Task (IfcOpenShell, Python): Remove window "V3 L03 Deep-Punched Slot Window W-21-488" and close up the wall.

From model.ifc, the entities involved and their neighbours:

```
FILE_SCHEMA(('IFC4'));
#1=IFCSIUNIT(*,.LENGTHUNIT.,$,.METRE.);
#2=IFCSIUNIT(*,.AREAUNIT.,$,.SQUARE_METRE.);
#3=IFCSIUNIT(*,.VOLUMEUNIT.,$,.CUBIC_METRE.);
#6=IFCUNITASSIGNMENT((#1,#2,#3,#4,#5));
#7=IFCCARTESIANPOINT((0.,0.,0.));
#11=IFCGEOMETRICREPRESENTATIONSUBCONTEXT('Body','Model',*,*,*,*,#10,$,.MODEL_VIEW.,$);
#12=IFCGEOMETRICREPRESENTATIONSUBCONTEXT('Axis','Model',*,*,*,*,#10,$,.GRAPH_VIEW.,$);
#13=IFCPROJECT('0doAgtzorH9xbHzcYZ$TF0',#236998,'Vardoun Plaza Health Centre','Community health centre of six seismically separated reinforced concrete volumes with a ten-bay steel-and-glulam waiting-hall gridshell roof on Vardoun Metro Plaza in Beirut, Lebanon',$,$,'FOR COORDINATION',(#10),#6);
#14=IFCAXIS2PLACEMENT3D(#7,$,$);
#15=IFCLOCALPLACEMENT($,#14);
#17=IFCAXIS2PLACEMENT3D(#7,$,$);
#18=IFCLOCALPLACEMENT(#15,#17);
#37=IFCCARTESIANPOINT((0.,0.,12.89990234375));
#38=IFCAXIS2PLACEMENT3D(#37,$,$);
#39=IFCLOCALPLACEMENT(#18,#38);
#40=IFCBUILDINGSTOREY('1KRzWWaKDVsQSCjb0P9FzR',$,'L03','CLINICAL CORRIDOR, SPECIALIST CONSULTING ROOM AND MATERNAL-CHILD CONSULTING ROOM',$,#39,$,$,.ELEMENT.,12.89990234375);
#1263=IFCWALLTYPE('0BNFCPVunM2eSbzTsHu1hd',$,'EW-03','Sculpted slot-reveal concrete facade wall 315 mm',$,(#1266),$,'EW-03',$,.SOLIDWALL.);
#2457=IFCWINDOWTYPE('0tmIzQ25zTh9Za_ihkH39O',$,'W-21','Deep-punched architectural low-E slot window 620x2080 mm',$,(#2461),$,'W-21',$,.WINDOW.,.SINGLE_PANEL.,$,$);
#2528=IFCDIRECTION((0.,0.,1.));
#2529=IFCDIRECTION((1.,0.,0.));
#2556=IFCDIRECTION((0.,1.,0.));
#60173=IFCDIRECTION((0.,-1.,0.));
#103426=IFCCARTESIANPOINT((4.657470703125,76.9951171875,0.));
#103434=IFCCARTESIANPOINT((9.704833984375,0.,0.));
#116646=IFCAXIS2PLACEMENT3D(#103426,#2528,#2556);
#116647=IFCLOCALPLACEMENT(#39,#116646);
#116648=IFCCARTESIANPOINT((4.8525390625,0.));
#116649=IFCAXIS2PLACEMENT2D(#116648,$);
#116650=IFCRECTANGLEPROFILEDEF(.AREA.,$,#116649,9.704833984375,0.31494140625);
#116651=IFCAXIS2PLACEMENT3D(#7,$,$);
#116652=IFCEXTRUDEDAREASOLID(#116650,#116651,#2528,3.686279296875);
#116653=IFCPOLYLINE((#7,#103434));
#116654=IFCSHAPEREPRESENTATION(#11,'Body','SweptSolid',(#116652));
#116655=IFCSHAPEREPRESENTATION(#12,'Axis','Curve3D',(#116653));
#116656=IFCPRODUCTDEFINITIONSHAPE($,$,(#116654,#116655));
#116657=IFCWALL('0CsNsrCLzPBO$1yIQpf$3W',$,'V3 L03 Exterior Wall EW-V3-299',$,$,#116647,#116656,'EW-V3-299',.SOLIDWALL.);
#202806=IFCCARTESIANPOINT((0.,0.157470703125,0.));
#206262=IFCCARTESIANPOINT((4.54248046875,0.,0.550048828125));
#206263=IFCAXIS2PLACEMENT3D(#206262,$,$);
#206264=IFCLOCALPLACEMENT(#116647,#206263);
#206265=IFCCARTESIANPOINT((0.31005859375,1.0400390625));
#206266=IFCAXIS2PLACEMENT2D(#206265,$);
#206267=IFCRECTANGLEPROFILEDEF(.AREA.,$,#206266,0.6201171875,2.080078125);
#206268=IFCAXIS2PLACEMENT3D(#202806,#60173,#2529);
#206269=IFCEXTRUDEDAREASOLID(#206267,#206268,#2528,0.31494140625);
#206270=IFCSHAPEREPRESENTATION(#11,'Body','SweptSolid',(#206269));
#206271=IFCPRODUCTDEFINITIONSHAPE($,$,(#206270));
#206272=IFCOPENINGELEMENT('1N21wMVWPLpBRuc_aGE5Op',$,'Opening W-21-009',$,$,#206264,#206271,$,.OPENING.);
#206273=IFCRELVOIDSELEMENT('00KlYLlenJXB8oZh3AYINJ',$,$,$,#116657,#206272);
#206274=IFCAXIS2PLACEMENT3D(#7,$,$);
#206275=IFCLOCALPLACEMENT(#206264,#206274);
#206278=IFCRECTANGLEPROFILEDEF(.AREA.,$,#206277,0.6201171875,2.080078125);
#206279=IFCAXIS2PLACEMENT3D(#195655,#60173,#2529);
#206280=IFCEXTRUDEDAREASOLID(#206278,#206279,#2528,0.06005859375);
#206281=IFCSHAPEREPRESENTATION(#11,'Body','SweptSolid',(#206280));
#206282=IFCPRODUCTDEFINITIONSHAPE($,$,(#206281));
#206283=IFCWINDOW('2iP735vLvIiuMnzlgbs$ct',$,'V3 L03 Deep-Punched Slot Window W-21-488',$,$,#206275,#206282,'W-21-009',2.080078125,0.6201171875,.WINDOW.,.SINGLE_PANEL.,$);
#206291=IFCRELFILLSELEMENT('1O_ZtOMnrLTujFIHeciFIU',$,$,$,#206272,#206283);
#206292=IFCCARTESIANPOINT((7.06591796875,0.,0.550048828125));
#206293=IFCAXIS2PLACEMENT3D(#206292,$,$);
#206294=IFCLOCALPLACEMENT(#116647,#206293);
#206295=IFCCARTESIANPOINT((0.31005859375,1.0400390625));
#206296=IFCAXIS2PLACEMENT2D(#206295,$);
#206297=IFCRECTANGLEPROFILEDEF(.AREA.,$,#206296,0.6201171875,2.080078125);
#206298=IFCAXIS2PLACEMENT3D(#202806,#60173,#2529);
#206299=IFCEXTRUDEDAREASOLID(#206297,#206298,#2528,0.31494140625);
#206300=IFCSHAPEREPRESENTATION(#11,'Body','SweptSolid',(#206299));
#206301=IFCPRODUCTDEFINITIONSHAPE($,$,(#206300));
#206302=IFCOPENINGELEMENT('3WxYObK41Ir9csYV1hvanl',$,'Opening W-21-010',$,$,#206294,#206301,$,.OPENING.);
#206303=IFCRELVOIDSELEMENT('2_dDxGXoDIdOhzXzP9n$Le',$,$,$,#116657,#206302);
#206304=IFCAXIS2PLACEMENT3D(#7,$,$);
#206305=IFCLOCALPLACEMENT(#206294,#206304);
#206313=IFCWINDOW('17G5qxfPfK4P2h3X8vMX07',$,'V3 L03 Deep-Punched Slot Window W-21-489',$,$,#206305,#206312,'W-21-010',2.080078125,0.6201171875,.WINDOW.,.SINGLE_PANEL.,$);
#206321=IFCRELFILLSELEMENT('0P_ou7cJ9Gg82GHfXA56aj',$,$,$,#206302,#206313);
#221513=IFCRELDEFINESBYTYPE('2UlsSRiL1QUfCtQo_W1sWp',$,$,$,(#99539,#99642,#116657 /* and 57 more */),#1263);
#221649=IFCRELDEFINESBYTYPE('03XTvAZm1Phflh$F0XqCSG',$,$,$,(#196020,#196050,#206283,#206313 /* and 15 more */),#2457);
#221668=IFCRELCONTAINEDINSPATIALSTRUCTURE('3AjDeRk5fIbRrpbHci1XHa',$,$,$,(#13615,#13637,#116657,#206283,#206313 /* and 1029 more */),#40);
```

```python
import ifcopenshell
import ifcopenshell.api.feature
import ifcopenshell.api.root
import ifcopenshell.geom
import ifcopenshell.util.shape

model = ifcopenshell.open("model.ifc")
settings = ifcopenshell.geom.settings()


def volume(element):
    """Net volume in cubic metres, openings subtracted."""
    shape = ifcopenshell.geom.create_shape(settings, element)
    return ifcopenshell.util.shape.get_volume(shape.geometry)


window = model.by_guid("2iP735vLvIiuMnzlgbs$ct")
opening = window.FillsVoids[0].RelatingOpeningElement
wall = opening.VoidsElements[0].RelatingBuildingElement
before = volume(wall)

ifcopenshell.api.root.remove_product(model, product=window)
ifcopenshell.api.feature.remove_feature(model, feature=opening)

after = volume(wall)

print(f"wall volume {before:.3f} -> {after:.3f} m3")

model.write("model_v2.ifc")
```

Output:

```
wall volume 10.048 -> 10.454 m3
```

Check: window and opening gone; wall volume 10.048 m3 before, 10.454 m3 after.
